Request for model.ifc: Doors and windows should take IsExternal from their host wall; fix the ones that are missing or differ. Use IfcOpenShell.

First a look at what the model holds.

```python
import ifcopenshell
import ifcopenshell.util.element

model = ifcopenshell.open("model.ifc")
print(model.schema)
seen = {}
for e in model.by_type("IfcDoor") + model.by_type("IfcWindow"):
    if not e.FillsVoids:
        continue
    host = e.FillsVoids[0].RelatingOpeningElement.VoidsElements[0].RelatingBuildingElement
    own = ifcopenshell.util.element.get_pset(e, f"Pset_{e.is_a()[3:].removesuffix('StandardCase')}Common", "IsExternal")
    wall = ifcopenshell.util.element.get_pset(host, "Pset_WallCommon", "IsExternal")
    seen[e.is_a(), own, wall] = seen.get((e.is_a(), own, wall), 0) + 1
for (cls, own, wall), count in sorted(seen.items(), key=str):
    print(count, cls, "IsExternal:", own, "| host wall:", wall)
```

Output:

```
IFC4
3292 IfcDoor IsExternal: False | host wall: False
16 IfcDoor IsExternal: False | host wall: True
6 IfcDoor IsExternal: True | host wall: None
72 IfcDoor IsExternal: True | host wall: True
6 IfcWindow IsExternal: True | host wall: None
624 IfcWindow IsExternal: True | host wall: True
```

```python
import ifcopenshell
import ifcopenshell.api.pset
import ifcopenshell.util.element

model = ifcopenshell.open("model.ifc")

count = 0
for ifc_class, pset_name in (("IfcDoor", "Pset_DoorCommon"), ("IfcWindow", "Pset_WindowCommon")):
    for e in model.by_type(ifc_class):
        if not e.FillsVoids:
            continue
        host = e.FillsVoids[0].RelatingOpeningElement.VoidsElements[0].RelatingBuildingElement
        external = ifcopenshell.util.element.get_pset(host, "Pset_WallCommon", "IsExternal")
        if external is None or ifcopenshell.util.element.get_pset(e, pset_name, "IsExternal") == external:
            continue
        pset = ifcopenshell.api.pset.add_pset(model, product=e, name=pset_name)
        ifcopenshell.api.pset.edit_pset(model, pset=pset, properties={"IsExternal": external})
        count += 1

print(count, "updated")

model.write("model_rev.ifc")
```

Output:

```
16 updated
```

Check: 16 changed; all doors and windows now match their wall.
